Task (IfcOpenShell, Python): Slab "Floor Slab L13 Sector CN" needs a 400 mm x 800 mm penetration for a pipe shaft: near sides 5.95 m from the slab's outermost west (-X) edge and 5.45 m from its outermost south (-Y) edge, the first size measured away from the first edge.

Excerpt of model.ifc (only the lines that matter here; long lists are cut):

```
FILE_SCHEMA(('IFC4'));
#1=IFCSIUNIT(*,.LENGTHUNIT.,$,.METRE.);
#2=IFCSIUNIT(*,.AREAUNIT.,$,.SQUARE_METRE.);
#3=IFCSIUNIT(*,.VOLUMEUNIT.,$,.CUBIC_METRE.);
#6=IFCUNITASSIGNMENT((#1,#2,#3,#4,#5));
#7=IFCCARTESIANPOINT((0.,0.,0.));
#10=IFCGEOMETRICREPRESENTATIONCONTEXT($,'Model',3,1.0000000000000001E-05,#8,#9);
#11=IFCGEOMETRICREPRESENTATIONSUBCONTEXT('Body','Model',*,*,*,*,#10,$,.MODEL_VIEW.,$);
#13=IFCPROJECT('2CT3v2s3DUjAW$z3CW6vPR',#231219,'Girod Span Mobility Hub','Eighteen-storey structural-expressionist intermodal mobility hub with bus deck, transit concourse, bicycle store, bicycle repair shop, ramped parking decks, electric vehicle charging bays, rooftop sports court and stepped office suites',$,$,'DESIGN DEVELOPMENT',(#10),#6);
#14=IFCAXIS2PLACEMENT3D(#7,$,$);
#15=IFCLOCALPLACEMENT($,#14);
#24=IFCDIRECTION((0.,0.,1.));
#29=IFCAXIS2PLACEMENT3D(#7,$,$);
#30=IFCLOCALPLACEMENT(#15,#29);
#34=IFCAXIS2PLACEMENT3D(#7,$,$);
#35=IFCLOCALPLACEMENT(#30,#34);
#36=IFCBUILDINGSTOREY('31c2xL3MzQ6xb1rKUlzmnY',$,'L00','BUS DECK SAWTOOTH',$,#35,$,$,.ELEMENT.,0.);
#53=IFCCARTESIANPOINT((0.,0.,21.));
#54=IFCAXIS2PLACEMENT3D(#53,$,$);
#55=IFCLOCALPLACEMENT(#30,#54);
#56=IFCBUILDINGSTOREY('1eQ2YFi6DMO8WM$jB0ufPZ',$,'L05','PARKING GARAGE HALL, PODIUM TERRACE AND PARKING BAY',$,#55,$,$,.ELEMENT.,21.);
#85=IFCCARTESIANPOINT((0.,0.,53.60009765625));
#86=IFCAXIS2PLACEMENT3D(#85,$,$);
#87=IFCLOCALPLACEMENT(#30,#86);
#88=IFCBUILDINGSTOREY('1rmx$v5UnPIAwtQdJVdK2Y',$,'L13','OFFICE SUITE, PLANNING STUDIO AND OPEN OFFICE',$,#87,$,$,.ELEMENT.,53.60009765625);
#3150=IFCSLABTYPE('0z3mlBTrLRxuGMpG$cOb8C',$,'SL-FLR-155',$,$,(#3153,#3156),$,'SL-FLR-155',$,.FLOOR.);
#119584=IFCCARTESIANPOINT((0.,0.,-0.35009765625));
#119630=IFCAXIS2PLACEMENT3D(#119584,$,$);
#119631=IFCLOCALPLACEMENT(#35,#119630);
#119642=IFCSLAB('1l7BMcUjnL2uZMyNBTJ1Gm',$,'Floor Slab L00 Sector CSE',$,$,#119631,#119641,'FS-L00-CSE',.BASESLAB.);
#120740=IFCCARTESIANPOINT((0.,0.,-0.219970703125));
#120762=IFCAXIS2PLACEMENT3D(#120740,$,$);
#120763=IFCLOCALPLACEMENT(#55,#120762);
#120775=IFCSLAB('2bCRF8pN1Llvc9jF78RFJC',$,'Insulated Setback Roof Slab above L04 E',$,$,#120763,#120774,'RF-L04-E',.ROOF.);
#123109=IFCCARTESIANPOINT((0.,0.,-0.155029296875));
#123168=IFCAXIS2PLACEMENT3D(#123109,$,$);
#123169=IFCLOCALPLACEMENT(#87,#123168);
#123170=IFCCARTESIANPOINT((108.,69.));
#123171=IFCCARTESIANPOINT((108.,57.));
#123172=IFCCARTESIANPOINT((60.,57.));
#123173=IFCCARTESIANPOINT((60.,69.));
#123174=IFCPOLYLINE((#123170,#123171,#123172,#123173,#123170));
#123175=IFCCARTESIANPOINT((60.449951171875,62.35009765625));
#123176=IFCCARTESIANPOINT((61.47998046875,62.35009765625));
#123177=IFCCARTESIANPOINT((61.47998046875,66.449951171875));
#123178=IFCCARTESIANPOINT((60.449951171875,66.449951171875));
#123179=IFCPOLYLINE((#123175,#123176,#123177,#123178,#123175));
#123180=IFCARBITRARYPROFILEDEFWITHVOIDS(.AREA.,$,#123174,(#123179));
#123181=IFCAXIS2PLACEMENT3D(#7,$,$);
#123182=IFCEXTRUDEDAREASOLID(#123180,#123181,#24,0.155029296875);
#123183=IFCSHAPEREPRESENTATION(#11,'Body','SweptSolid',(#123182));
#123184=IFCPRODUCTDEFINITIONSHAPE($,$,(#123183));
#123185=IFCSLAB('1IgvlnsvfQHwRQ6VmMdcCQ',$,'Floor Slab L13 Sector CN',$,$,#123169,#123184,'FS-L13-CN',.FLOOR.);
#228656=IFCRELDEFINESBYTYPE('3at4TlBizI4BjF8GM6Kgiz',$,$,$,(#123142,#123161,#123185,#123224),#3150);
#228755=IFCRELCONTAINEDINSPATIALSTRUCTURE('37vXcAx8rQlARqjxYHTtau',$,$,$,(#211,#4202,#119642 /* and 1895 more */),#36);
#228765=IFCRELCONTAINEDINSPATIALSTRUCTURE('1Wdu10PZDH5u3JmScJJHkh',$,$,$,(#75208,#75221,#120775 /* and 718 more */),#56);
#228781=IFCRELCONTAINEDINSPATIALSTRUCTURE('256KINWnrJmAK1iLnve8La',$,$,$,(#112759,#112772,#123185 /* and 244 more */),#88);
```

```python
import numpy as np
import ifcopenshell
import ifcopenshell.api.feature
import ifcopenshell.api.geometry
import ifcopenshell.api.root
import ifcopenshell.geom
import ifcopenshell.util.placement
import ifcopenshell.util.representation
import ifcopenshell.util.shape
import ifcopenshell.util.unit

model = ifcopenshell.open("model.ifc")
unit_scale = ifcopenshell.util.unit.calculate_unit_scale(model)
settings = ifcopenshell.geom.settings()


def volume(element):
    """Net volume in cubic metres, openings subtracted."""
    shape = ifcopenshell.geom.create_shape(settings, element)
    return ifcopenshell.util.shape.get_volume(shape.geometry)


slab = model.by_id(123185)
before = volume(slab)

# Extent in the slab's own axes, in metres. The edges named are its -X and -Y sides.
slab_shape = ifcopenshell.geom.create_shape(settings, slab)
vertices = ifcopenshell.util.shape.get_vertices(slab_shape.geometry)
x_min, y_min, bottom = vertices.min(axis=0)
top = vertices[:, 2].max()

opening = ifcopenshell.api.root.create_entity(model, ifc_class="IfcOpeningElement", name="Pipe shaft opening", predefined_type="OPENING")
context = ifcopenshell.util.representation.get_context(model, "Model", "Body", "MODEL_VIEW")
width, depth = 0.4, 0.8
outline = [(0.0, 0.0), (width, 0.0), (width, depth), (0.0, depth), (0.0, 0.0)]
# Overshoot both faces by 50 mm so the cut is clean.
shape = ifcopenshell.api.geometry.add_slab_representation(
    model, context=context, depth=top - bottom + 0.1, polyline=outline
)
ifcopenshell.api.geometry.assign_representation(model, product=opening, representation=shape)

matrix = ifcopenshell.util.placement.get_local_placement(slab.ObjectPlacement)
matrix[:, 3] = matrix @ np.append(np.array([x_min + 5.95, y_min + 5.45, bottom - 0.05]) / unit_scale, 1.0)
ifcopenshell.api.geometry.edit_object_placement(model, product=opening, matrix=matrix, is_si=False)
ifcopenshell.api.feature.add_feature(model, feature=opening, element=slab)

after = volume(slab)

print(f"slab volume {before:.3f} -> {after:.3f} m3")

model.write("model_edited.ifc")
```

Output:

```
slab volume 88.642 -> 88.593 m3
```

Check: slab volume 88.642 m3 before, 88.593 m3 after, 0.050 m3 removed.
